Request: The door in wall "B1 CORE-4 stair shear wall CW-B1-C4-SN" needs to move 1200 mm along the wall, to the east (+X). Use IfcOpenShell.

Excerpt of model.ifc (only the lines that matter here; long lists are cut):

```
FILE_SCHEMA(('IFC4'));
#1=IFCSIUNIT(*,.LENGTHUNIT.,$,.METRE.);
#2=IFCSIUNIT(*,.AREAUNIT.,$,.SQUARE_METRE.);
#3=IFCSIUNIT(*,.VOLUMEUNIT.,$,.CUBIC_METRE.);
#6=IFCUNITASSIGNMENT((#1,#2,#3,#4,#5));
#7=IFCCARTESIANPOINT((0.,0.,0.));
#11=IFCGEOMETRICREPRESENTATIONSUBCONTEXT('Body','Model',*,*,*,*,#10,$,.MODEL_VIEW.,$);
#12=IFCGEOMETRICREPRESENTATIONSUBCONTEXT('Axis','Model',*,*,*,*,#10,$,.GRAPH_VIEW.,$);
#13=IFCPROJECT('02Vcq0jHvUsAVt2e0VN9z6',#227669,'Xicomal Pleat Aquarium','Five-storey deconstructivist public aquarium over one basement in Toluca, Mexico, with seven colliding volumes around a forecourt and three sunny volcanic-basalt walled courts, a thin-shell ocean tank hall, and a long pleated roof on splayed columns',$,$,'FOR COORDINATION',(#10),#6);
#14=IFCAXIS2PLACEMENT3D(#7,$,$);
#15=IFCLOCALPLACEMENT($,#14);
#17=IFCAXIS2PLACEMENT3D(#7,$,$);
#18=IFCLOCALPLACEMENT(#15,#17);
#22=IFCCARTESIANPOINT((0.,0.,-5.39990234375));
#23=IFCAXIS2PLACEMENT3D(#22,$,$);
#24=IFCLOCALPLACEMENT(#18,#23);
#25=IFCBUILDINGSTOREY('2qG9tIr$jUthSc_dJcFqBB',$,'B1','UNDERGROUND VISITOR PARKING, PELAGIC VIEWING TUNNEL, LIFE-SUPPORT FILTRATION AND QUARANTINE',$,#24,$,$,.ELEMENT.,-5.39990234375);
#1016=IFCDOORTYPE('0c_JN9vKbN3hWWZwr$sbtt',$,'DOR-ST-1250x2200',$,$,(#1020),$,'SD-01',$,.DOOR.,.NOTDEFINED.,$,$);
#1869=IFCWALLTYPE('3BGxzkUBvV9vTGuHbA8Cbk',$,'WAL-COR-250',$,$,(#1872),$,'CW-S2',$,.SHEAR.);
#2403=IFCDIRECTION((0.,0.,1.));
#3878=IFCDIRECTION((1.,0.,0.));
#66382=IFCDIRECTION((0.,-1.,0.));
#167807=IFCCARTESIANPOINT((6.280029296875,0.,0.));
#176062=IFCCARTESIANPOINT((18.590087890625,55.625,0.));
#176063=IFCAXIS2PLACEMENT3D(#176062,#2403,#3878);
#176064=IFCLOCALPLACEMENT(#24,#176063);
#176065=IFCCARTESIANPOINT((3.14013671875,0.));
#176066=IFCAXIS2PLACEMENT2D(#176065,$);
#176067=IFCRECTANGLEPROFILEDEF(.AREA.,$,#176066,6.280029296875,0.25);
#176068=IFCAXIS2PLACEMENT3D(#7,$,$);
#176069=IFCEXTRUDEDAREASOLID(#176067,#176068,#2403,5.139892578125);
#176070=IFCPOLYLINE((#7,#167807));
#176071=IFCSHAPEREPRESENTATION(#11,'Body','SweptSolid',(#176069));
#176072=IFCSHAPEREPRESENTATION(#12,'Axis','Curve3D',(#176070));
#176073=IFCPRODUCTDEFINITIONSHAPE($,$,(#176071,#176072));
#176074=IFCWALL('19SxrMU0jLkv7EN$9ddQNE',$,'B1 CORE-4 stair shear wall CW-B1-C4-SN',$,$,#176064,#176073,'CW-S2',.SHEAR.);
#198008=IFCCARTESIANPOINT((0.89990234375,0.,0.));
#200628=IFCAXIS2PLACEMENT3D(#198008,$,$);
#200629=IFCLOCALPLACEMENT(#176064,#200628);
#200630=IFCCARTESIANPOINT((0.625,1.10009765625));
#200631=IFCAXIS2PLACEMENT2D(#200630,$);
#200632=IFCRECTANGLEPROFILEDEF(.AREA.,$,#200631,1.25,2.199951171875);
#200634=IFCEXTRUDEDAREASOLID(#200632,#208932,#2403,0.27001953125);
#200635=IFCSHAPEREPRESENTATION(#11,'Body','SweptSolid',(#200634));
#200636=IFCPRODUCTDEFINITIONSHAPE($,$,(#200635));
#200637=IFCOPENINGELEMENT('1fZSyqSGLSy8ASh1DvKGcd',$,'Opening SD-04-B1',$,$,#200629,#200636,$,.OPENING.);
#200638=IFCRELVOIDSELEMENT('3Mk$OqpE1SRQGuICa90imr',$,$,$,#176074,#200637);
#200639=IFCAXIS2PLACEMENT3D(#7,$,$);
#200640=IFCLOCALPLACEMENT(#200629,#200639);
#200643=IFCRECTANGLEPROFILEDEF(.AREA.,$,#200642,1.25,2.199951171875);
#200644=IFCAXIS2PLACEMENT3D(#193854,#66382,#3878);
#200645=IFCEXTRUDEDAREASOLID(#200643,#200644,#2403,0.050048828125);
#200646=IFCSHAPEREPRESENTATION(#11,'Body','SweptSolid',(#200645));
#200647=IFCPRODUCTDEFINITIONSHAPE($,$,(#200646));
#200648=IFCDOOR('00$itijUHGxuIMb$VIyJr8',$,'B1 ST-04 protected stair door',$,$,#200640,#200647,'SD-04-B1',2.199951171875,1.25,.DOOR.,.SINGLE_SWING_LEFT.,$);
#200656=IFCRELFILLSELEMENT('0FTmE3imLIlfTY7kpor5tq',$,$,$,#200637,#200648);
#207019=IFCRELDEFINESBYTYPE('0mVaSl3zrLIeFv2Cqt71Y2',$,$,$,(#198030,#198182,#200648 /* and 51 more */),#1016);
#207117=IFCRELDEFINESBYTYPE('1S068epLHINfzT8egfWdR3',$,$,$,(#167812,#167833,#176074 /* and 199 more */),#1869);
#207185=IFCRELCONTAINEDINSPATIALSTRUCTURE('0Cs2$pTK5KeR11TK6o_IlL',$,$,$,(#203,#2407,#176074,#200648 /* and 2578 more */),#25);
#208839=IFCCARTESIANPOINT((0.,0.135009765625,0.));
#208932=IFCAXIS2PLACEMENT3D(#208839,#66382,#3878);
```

```python
import ifcopenshell
import ifcopenshell.api.geometry
import ifcopenshell.util.placement

model = ifcopenshell.open("model.ifc")

door = model.by_id(200648)
opening = door.FillsVoids[0].RelatingOpeningElement
wall = opening.VoidsElements[0].RelatingBuildingElement

wall_matrix = ifcopenshell.util.placement.get_local_placement(wall.ObjectPlacement)
shift = wall_matrix[:3, 0] * 1.2
before = ifcopenshell.util.placement.get_local_placement(door.ObjectPlacement)[:3, 3].copy()

# The door is placed relative to its opening, so it follows when the opening moves.
matrix = ifcopenshell.util.placement.get_local_placement(opening.ObjectPlacement)
matrix[:3, 3] += shift
ifcopenshell.api.geometry.edit_object_placement(
    model, product=opening, matrix=matrix, is_si=False, should_transform_children=True
)

after = ifcopenshell.util.placement.get_local_placement(door.ObjectPlacement)[:3, 3]
print("door moved by", (after - before).round(3) + 0.0)

model.write("model_rev.ifc")
```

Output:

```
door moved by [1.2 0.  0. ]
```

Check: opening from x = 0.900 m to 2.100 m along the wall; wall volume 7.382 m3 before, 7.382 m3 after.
